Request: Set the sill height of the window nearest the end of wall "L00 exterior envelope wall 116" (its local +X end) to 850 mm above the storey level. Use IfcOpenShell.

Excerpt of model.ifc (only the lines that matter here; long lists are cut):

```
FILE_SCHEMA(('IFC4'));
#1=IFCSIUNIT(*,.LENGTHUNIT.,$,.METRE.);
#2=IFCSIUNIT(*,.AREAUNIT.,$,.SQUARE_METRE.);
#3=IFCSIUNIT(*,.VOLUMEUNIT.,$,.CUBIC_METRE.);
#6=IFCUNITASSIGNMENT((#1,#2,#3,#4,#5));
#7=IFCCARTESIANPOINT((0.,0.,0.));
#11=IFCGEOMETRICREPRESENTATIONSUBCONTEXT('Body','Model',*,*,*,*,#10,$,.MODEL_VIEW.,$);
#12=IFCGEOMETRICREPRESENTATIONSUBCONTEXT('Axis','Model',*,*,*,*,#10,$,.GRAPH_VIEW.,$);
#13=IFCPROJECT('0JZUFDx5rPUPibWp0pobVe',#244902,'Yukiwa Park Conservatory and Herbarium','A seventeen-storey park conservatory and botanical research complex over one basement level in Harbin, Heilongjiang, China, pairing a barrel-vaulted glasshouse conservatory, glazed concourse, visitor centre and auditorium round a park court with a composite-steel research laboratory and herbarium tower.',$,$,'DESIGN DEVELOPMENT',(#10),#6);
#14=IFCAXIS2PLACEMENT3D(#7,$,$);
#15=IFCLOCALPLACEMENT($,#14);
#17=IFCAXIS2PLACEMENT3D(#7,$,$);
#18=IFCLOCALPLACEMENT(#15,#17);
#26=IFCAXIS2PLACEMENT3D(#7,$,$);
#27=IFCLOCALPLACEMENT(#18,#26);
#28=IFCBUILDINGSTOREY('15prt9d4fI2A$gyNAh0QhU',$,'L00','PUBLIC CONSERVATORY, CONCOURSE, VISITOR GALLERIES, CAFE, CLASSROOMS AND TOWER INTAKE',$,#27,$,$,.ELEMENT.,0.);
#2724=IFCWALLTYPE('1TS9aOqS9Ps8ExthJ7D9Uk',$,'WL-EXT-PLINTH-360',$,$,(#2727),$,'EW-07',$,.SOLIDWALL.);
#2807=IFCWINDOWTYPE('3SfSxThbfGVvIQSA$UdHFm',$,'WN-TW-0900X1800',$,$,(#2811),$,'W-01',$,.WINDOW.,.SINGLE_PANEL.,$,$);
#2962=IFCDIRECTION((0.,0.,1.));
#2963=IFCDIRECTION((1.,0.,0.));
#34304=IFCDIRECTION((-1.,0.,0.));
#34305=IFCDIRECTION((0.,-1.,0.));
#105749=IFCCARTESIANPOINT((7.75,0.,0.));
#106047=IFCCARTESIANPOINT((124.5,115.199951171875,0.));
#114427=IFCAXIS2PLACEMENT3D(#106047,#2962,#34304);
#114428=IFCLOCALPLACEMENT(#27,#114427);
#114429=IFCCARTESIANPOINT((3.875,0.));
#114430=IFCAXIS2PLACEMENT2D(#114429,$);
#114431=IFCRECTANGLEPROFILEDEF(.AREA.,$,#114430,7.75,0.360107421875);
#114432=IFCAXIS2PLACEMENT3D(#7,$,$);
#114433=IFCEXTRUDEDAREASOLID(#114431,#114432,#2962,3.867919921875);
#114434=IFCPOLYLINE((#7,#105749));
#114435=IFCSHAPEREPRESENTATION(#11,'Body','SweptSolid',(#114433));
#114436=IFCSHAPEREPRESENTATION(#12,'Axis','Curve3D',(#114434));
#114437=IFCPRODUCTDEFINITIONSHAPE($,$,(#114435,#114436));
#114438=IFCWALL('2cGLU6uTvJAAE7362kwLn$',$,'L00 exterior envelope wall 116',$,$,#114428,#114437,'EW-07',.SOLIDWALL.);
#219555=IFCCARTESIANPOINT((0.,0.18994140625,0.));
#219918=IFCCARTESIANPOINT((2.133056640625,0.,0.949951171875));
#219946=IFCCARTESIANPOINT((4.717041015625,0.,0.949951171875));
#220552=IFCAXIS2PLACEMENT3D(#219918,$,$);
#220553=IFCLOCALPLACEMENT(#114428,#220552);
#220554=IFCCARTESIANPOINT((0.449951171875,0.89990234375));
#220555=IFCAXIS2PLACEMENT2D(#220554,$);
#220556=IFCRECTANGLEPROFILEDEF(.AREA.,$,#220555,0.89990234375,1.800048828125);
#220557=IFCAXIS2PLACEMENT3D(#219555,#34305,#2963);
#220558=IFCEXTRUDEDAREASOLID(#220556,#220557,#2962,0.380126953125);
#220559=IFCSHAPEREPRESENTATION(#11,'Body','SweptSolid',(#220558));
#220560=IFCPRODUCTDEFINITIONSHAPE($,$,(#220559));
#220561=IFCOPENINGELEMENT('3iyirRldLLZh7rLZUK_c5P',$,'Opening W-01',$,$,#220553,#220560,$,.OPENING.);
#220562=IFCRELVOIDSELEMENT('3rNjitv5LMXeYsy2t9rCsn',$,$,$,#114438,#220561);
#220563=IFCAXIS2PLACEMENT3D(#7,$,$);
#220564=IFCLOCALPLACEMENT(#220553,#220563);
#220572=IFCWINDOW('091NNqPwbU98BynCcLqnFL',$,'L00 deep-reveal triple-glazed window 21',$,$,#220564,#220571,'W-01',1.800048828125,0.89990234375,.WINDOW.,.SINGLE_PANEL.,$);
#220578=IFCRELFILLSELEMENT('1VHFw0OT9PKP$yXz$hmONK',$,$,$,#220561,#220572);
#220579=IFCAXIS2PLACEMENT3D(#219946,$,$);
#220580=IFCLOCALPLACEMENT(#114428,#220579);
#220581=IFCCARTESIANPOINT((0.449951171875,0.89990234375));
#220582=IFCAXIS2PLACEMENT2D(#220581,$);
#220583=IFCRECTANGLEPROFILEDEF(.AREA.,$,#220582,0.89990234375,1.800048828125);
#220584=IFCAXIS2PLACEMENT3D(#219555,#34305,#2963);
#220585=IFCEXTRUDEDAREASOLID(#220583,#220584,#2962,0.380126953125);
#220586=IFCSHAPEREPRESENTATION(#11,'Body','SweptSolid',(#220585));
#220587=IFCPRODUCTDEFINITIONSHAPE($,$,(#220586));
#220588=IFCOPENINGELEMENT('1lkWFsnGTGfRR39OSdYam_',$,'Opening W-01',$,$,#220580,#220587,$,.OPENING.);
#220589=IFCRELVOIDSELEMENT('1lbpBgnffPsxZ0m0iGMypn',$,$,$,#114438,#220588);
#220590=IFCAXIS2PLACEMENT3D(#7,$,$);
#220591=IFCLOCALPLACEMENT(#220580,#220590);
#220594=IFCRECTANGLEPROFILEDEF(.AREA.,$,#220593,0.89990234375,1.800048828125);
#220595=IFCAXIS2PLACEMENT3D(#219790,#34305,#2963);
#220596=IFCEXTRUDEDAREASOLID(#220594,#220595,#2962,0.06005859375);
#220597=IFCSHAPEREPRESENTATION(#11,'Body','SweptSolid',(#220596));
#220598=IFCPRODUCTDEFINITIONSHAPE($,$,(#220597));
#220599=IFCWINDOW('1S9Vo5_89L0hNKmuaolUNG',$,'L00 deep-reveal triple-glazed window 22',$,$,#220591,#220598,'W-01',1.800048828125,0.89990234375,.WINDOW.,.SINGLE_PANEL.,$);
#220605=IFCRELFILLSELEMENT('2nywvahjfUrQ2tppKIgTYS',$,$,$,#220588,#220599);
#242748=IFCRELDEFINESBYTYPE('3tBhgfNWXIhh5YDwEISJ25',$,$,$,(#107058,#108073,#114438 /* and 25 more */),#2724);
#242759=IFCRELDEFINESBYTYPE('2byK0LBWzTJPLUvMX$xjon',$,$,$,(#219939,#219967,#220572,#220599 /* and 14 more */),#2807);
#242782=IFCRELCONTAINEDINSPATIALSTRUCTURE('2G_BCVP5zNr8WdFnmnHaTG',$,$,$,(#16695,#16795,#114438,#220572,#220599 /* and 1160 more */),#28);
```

```python
import numpy as np
import ifcopenshell
import ifcopenshell.api.geometry
import ifcopenshell.geom
import ifcopenshell.util.element
import ifcopenshell.util.placement
import ifcopenshell.util.shape
import ifcopenshell.util.unit

model = ifcopenshell.open("model.ifc")
unit_scale = ifcopenshell.util.unit.calculate_unit_scale(model)

window = model.by_guid("1S9Vo5_89L0hNKmuaolUNG")
opening = window.FillsVoids[0].RelatingOpeningElement
storey = ifcopenshell.util.element.get_container(window, ifc_class="IfcBuildingStorey")
level = ifcopenshell.util.placement.get_local_placement(storey.ObjectPlacement)[2, 3]

# The opening's origin need not be at the sill, so measure its lowest point.
shape = ifcopenshell.geom.create_shape(ifcopenshell.geom.settings(), opening)
bottom = ifcopenshell.util.shape.get_shape_bottom_elevation(shape, shape.geometry) / unit_scale
dz = level + 0.85 / unit_scale - bottom

shift = np.array([0.0, 0.0, dz])
# The window is placed relative to its opening, so it follows when the opening moves.
matrix = ifcopenshell.util.placement.get_local_placement(opening.ObjectPlacement)
matrix[:3, 3] += shift
ifcopenshell.api.geometry.edit_object_placement(
    model, product=opening, matrix=matrix, is_si=False, should_transform_children=True
)

print(f"moved by {dz * unit_scale:+.3f} m")

model.write("model_rev.ifc")
```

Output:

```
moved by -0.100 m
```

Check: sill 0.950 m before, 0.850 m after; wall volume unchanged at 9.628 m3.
